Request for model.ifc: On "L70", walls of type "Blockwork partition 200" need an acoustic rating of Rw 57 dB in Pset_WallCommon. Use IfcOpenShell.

First a look at what the model holds.

```python
import ifcopenshell
import ifcopenshell.util.element

model = ifcopenshell.open("model.ifc")
print(model.schema)
storey = next(s for s in model.by_type("IfcBuildingStorey") if s.Name == "L70")
walls = [e for e in ifcopenshell.util.element.get_decomposition(storey) if e.is_a("IfcWall")]
seen = {}
for e in walls:
    element_type = ifcopenshell.util.element.get_type(e)
    key = (element_type.Name if element_type != e and element_type else None, ifcopenshell.util.element.get_pset(e, "Pset_WallCommon", "AcousticRating"))
    seen[key] = seen.get(key, 0) + 1
for (name, value), count in sorted(seen.items(), key=str):
    print(count, "x", name, "|", value)
```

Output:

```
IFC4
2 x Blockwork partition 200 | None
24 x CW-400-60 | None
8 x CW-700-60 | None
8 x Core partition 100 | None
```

```python
import ifcopenshell
import ifcopenshell.api.pset
import ifcopenshell.util.element

model = ifcopenshell.open("model.ifc")

storey = next(s for s in model.by_type("IfcBuildingStorey") if s.Name == "L70")
walls = [e for e in ifcopenshell.util.element.get_decomposition(storey) if e.is_a("IfcWall")]

count = 0
for e in walls:
    element_type = ifcopenshell.util.element.get_type(e)
    if element_type in (None, e) or element_type.Name != "Blockwork partition 200":
        continue
    found = ifcopenshell.util.element.get_pset(e, "Pset_WallCommon", should_inherit=False)
    if found:
        pset = model.by_id(found["id"])
        if len(ifcopenshell.util.element.get_elements_by_pset(pset)) > 1:
            pset = ifcopenshell.api.pset.unshare_pset(model, products=[e], pset=pset)[0]
    else:
        pset = ifcopenshell.api.pset.add_pset(model, product=e, name="Pset_WallCommon")
    ifcopenshell.api.pset.edit_pset(model, pset=pset, properties={"AcousticRating": "Rw 57 dB"})
    count += 1

print(count, "walls updated")

model.write("model_updated.ifc")
```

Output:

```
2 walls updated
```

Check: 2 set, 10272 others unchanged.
